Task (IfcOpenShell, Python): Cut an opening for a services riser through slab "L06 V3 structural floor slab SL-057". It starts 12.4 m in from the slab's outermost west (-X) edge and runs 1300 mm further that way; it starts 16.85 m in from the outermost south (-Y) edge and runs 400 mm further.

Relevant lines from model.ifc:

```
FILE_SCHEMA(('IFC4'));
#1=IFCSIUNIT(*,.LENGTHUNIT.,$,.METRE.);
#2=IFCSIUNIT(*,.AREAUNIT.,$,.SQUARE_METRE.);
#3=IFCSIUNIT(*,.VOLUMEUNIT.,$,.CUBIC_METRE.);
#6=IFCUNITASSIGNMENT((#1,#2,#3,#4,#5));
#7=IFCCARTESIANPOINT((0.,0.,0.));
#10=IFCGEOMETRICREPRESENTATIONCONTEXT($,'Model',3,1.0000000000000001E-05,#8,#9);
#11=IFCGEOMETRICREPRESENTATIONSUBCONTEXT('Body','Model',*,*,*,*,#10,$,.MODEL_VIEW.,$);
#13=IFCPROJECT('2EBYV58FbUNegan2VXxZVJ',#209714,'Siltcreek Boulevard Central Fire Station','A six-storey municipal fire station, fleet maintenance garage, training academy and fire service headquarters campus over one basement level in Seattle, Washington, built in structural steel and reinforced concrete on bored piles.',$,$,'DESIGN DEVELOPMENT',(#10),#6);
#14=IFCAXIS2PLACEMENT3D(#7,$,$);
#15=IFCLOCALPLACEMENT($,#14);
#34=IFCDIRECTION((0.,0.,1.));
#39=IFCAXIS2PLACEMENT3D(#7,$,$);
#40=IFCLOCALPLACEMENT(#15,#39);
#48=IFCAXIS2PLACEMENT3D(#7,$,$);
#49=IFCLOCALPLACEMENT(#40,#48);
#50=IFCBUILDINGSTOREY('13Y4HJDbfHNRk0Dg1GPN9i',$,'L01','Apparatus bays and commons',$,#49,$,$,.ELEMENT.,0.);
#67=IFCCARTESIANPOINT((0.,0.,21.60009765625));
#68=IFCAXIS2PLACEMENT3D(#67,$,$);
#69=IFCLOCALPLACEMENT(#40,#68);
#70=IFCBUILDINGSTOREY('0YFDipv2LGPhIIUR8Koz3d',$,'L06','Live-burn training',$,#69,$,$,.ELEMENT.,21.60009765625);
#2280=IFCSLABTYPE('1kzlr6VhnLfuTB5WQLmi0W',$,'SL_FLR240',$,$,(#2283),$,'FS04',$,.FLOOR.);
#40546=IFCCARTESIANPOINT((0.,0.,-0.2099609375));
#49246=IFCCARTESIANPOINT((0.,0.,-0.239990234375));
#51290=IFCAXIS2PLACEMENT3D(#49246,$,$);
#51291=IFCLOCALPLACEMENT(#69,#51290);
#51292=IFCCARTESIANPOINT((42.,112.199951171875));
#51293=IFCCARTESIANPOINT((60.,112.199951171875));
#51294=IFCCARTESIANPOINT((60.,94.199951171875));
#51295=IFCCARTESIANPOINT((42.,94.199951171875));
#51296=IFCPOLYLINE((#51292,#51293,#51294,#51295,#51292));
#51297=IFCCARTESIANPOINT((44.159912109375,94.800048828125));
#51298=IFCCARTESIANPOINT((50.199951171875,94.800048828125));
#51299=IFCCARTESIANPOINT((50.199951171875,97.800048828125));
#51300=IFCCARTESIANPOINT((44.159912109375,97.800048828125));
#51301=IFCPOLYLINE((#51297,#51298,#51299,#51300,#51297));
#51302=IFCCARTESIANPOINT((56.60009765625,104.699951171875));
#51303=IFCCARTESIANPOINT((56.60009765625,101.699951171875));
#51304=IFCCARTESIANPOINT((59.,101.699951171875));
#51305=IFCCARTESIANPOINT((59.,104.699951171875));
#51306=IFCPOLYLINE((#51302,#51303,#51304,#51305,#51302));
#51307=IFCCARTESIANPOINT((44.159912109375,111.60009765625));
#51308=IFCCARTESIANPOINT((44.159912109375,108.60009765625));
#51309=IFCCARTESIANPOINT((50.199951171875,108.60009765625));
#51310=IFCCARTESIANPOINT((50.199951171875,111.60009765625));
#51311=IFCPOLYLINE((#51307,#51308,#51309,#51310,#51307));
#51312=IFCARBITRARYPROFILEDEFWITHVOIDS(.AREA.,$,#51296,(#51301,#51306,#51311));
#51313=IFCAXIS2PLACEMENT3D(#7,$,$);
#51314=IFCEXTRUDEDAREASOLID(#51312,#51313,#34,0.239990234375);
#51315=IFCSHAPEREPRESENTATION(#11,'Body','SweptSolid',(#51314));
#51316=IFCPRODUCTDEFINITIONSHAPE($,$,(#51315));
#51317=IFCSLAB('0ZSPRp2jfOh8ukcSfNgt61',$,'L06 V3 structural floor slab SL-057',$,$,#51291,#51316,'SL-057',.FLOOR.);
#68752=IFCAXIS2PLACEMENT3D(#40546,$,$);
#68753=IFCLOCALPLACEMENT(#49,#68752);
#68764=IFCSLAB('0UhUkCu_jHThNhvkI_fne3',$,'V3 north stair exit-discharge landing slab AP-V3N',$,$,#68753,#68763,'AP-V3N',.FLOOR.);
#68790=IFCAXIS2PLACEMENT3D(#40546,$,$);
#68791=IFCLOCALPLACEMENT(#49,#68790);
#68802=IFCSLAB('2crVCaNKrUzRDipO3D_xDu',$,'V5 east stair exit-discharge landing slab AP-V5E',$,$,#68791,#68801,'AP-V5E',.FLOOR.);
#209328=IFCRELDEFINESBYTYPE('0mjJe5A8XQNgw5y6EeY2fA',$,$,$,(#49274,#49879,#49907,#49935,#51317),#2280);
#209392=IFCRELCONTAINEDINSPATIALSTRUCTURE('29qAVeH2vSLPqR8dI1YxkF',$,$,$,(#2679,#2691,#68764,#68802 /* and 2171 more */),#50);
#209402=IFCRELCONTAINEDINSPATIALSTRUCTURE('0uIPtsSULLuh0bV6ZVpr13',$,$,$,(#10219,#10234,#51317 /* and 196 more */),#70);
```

```python
import numpy as np
import ifcopenshell
import ifcopenshell.api.feature
import ifcopenshell.api.geometry
import ifcopenshell.api.root
import ifcopenshell.geom
import ifcopenshell.util.placement
import ifcopenshell.util.representation
import ifcopenshell.util.shape
import ifcopenshell.util.unit

model = ifcopenshell.open("model.ifc")
unit_scale = ifcopenshell.util.unit.calculate_unit_scale(model)
settings = ifcopenshell.geom.settings()


def volume(element):
    """Net volume in cubic metres, openings subtracted."""
    shape = ifcopenshell.geom.create_shape(settings, element)
    return ifcopenshell.util.shape.get_volume(shape.geometry)


slab = model.by_guid("0ZSPRp2jfOh8ukcSfNgt61")
before = volume(slab)

# Extent in the slab's own axes, in metres. The edges named are its -X and -Y sides.
slab_shape = ifcopenshell.geom.create_shape(settings, slab)
vertices = ifcopenshell.util.shape.get_vertices(slab_shape.geometry)
x_min, y_min, bottom = vertices.min(axis=0)
top = vertices[:, 2].max()

opening = ifcopenshell.api.root.create_entity(model, ifc_class="IfcOpeningElement", name="Services riser opening", predefined_type="OPENING")
context = ifcopenshell.util.representation.get_context(model, "Model", "Body", "MODEL_VIEW")
width, depth = 1.3, 0.4
outline = [(0.0, 0.0), (width, 0.0), (width, depth), (0.0, depth), (0.0, 0.0)]
# Overshoot both faces by 50 mm so the cut is clean.
shape = ifcopenshell.api.geometry.add_slab_representation(
    model, context=context, depth=top - bottom + 0.1, polyline=outline
)
ifcopenshell.api.geometry.assign_representation(model, product=opening, representation=shape)

matrix = ifcopenshell.util.placement.get_local_placement(slab.ObjectPlacement)
matrix[:, 3] = matrix @ np.append(np.array([x_min + 12.4, y_min + 16.85, bottom - 0.05]) / unit_scale, 1.0)
ifcopenshell.api.geometry.edit_object_placement(model, product=opening, matrix=matrix, is_si=False)
ifcopenshell.api.feature.add_feature(model, feature=opening, element=slab)

after = volume(slab)

print(f"slab volume {before:.3f} -> {after:.3f} m3")

model.write("model_updated.ifc")
```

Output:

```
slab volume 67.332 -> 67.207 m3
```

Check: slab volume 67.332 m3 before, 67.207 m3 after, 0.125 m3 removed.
